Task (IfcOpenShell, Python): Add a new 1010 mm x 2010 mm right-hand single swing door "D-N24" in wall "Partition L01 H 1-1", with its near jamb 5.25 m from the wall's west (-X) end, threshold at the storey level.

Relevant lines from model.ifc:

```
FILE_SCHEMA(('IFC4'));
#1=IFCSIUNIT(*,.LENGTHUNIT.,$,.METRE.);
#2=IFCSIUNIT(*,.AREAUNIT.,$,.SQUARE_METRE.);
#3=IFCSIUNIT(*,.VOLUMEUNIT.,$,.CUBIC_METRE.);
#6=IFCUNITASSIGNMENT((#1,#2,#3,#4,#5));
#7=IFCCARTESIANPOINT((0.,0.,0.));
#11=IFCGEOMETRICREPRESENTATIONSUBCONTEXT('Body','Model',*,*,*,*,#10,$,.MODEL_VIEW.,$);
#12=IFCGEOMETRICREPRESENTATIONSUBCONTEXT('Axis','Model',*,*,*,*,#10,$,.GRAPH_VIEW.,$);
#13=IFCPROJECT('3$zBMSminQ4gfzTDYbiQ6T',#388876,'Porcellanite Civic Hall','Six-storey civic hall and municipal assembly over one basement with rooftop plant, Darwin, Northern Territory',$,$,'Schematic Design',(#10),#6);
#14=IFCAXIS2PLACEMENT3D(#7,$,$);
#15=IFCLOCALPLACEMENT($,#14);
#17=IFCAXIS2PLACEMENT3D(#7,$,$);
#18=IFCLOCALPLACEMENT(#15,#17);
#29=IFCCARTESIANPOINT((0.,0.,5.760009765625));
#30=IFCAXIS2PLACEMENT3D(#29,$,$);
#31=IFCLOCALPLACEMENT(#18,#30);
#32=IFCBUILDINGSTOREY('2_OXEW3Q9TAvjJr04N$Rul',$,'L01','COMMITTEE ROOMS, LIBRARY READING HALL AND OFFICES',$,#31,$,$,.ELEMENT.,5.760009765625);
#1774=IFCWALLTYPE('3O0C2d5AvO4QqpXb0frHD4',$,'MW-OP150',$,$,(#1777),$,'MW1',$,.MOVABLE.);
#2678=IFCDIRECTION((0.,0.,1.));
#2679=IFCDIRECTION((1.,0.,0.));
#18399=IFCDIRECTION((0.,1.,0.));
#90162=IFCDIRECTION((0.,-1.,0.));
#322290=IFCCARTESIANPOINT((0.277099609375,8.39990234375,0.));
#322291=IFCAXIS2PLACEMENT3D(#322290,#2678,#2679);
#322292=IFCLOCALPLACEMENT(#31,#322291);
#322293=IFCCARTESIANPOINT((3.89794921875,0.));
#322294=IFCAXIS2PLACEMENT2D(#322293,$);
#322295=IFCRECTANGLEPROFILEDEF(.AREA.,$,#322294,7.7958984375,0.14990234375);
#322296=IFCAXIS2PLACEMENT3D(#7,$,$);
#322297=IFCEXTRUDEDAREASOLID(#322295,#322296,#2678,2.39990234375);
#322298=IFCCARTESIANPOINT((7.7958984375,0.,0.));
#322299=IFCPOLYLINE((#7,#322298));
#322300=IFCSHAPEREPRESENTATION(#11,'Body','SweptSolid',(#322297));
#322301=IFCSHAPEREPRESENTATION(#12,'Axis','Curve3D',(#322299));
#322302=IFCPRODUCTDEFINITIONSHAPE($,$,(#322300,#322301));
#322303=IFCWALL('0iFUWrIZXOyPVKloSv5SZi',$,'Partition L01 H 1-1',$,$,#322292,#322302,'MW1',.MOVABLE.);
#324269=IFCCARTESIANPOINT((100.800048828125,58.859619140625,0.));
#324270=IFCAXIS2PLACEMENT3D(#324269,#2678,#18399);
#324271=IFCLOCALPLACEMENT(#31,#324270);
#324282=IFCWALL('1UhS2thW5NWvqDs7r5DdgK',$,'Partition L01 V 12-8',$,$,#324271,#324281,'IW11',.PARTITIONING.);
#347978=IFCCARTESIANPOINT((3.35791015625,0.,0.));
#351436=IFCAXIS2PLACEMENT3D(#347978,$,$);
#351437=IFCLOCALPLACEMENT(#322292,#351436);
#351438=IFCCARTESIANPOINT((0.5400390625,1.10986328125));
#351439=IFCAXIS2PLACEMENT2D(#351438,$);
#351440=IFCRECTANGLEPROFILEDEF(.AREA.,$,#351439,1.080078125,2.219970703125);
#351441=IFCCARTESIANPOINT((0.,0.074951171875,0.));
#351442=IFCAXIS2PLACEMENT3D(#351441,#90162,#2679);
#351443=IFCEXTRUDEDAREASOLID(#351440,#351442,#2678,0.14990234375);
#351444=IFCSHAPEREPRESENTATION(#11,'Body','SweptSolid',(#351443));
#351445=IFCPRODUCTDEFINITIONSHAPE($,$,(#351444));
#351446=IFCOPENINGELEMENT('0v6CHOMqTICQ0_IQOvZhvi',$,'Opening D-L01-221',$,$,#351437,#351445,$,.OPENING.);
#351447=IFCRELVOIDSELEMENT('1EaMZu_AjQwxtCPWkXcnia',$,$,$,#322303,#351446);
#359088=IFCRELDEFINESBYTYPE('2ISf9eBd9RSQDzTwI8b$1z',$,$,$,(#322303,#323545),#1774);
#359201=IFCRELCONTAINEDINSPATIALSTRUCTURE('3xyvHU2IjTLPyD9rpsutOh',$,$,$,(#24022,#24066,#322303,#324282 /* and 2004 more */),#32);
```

```python
import numpy as np
import ifcopenshell
import ifcopenshell.api.feature
import ifcopenshell.api.geometry
import ifcopenshell.api.root
import ifcopenshell.api.spatial
import ifcopenshell.geom
import ifcopenshell.util.element
import ifcopenshell.util.placement
import ifcopenshell.util.representation
import ifcopenshell.util.shape
import ifcopenshell.util.unit

model = ifcopenshell.open("model.ifc")
unit_scale = ifcopenshell.util.unit.calculate_unit_scale(model)
settings = ifcopenshell.geom.settings()


def volume(element):
    """Net volume in cubic metres, openings subtracted."""
    shape = ifcopenshell.geom.create_shape(settings, element)
    return ifcopenshell.util.shape.get_volume(shape.geometry)


wall = model.by_guid("0iFUWrIZXOyPVKloSv5SZi")
storey = ifcopenshell.util.element.get_container(wall, ifc_class="IfcBuildingStorey")
context = ifcopenshell.util.representation.get_context(model, "Model", "Body", "MODEL_VIEW")
before = volume(wall)

width, height, from_end, sill = 1.01, 2.01, 5.25, 0.0  # metres

# The wall runs along its own X axis, and the end named is its -X end.
wall_shape = ifcopenshell.geom.create_shape(settings, wall)
x, y, z = ifcopenshell.util.shape.get_vertices(wall_shape.geometry).T
start = x.min() + from_end
face, thickness = float(y.min()), float(y.max() - y.min())
wall_matrix = ifcopenshell.util.placement.get_local_placement(wall.ObjectPlacement)
level = ifcopenshell.util.placement.get_local_placement(storey.ObjectPlacement)[2, 3]


def in_wall(x, y):
    """Placement at x, y metres in the wall's axes, at sill height."""
    matrix = wall_matrix.copy()
    matrix[:, 3] = wall_matrix @ np.array([x / unit_scale, y / unit_scale, 0.0, 1.0])
    matrix[2, 3] = level + sill / unit_scale
    return matrix


# Opening: a box that overshoots both wall faces by 50 mm.
opening = ifcopenshell.api.root.create_entity(model, ifc_class="IfcOpeningElement", predefined_type="OPENING")
box = ifcopenshell.api.geometry.add_wall_representation(
    model, context=context, length=width, height=height, thickness=thickness + 0.1
)
ifcopenshell.api.geometry.assign_representation(model, product=opening, representation=box)
ifcopenshell.api.geometry.edit_object_placement(model, product=opening, matrix=in_wall(start, face - 0.05), is_si=False)
ifcopenshell.api.feature.add_feature(model, feature=opening, element=wall)

door = ifcopenshell.api.root.create_entity(model, ifc_class="IfcDoor", name="D-N24", predefined_type="DOOR")
door.OverallWidth, door.OverallHeight = width / unit_scale, height / unit_scale
door.OperationType = "SINGLE_SWING_RIGHT"
body = ifcopenshell.api.geometry.add_door_representation(
    model,
    context=context,
    overall_width=door.OverallWidth,
    overall_height=door.OverallHeight,
    operation_type="SINGLE_SWING_RIGHT",
    lining_properties={"LiningDepth": thickness / unit_scale, "ThresholdDepth": thickness / unit_scale},
)
ifcopenshell.api.geometry.assign_representation(model, product=door, representation=body)
ifcopenshell.api.spatial.assign_container(model, products=[door], relating_structure=storey)
ifcopenshell.api.feature.add_filling(model, opening=opening, element=door)

# The lining spans the wall, so the door starts at the wall face.
ifcopenshell.api.geometry.edit_object_placement(model, product=door, matrix=in_wall(start, face), is_si=False)

after = volume(wall)

print(f"wall volume {before:.3f} -> {after:.3f} m3")

model.write("model-out.ifc")
```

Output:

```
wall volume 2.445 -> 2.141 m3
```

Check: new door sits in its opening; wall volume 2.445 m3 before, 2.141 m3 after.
